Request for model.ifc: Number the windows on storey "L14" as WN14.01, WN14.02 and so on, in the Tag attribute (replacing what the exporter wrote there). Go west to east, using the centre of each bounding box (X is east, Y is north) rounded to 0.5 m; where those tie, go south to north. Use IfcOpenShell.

First a look at what the model holds.

```python
import ifcopenshell
import ifcopenshell.util.element
import ifcopenshell.util.placement

model = ifcopenshell.open("model.ifc")
print(model.schema)
storey = next(s for s in model.by_type("IfcBuildingStorey") if s.Name == "L14")
windows = [e for e in ifcopenshell.util.element.get_decomposition(storey) if e.is_a("IfcWindow")]
for e in sorted(windows, key=lambda e: e.id()):
    origin = ifcopenshell.util.placement.get_local_placement(e.ObjectPlacement)[:3, 3]
    print(e.id(), e.Tag, e.Name, origin.round(2) + 0.0, sep=" | ")
```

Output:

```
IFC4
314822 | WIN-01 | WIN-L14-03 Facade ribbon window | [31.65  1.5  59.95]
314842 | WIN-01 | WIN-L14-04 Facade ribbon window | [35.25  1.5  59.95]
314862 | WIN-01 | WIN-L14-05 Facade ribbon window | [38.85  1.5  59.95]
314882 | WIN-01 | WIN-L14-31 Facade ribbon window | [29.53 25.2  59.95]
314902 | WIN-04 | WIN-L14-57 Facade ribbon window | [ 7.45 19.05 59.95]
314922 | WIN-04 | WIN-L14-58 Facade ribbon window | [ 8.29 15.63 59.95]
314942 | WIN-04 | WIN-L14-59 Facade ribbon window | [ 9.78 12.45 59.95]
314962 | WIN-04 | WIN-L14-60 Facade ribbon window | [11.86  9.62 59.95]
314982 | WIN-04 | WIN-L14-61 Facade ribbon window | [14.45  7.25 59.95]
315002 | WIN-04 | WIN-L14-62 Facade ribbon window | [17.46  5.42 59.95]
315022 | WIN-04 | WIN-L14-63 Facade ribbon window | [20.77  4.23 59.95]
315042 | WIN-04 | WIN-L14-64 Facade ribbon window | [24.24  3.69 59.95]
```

```python
import ifcopenshell
import ifcopenshell.geom
import ifcopenshell.util.element
import ifcopenshell.util.shape

model = ifcopenshell.open("model.ifc")
settings = ifcopenshell.geom.settings()
settings.set("use-world-coords", True)


def centre(element):
    shape = ifcopenshell.geom.create_shape(settings, element)
    return ifcopenshell.util.shape.get_bbox_centroid(shape.geometry)


storey = next(s for s in model.by_type("IfcBuildingStorey") if s.Name == "L14")
windows = [e for e in ifcopenshell.util.element.get_decomposition(storey) if e.is_a("IfcWindow")]

# Insertion points can sit at a corner or the storey origin, so sort by the geometry (in metres).
centres = {e: centre(e) for e in windows}
windows.sort(key=lambda e: (round(centres[e][0] / 0.5), centres[e][1]))

for i, e in enumerate(windows, start=1):
    number = f"WN14.{i:02d}"
    e.Tag = number
    print(e.id(), number)

model.write("model-out.ifc")
```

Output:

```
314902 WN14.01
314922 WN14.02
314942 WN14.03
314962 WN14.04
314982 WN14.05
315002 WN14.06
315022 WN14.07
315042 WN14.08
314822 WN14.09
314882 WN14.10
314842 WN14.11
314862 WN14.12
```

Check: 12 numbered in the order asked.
